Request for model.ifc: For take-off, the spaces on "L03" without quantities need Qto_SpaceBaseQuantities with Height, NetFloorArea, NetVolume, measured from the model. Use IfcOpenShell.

First a look at what the model holds.

```python
import ifcopenshell
import ifcopenshell.util.element
import ifcopenshell.util.unit

model = ifcopenshell.open("model.ifc")
print(model.schema)
for unit_type in ("LENGTHUNIT", "AREAUNIT", "VOLUMEUNIT"):
    print(unit_type, ifcopenshell.util.unit.calculate_unit_scale(model, unit_type))
storey = next(s for s in model.by_type("IfcBuildingStorey") if s.Name == "L03")
spaces = [e for e in ifcopenshell.util.element.get_decomposition(storey) if e.is_a("IfcSpace")]
for e in sorted(spaces, key=lambda e: e.id()):
    print(e.id(), e.is_a(), e.Name, list(ifcopenshell.util.element.get_psets(e, qtos_only=True)), sep=" | ")
```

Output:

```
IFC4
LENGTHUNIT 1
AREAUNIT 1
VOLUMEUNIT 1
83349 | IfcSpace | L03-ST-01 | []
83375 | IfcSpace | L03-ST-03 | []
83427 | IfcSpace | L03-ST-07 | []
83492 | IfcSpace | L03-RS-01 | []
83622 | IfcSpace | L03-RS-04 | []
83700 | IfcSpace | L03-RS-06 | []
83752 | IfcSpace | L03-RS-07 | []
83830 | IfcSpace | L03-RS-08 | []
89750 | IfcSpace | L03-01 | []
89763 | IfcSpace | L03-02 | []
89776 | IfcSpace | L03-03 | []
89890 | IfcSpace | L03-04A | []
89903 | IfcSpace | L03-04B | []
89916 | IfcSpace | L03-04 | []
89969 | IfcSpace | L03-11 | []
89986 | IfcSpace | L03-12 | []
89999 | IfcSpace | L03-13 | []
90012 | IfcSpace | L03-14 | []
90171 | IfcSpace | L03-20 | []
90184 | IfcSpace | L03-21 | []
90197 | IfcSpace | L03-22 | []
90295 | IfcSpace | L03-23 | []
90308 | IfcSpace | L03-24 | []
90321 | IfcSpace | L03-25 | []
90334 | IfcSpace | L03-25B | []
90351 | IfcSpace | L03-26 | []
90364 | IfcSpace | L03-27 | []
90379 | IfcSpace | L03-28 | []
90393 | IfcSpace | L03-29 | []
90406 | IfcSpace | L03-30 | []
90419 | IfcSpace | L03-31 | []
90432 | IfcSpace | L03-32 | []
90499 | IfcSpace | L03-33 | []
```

```python
import ifcopenshell
import ifcopenshell.api.pset
import ifcopenshell.geom
import ifcopenshell.util.element
import ifcopenshell.util.shape
import ifcopenshell.util.unit

model = ifcopenshell.open("model.ifc")
unit_scale = ifcopenshell.util.unit.calculate_unit_scale(model)
area_scale = ifcopenshell.util.unit.calculate_unit_scale(model, "AREAUNIT")
volume_scale = ifcopenshell.util.unit.calculate_unit_scale(model, "VOLUMEUNIT")
settings = ifcopenshell.geom.settings()

storey = next(s for s in model.by_type("IfcBuildingStorey") if s.Name == "L03")
spaces = [e for e in ifcopenshell.util.element.get_decomposition(storey) if e.is_a("IfcSpace")]

for e in sorted(spaces, key=lambda e: e.id()):
    if ifcopenshell.util.element.get_psets(e, qtos_only=True, should_inherit=False):
        continue
    # Geometry comes back in metres, in the element's own axes.
    shape = ifcopenshell.geom.create_shape(settings, e)
    values = {
        "Height": ifcopenshell.util.shape.get_z(shape.geometry) / unit_scale,
        "NetFloorArea": ifcopenshell.util.shape.get_footprint_area(shape.geometry) / area_scale,
        "NetVolume": ifcopenshell.util.shape.get_volume(shape.geometry) / volume_scale,
    }
    qto = ifcopenshell.api.pset.add_qto(model, product=e, name="Qto_SpaceBaseQuantities")
    ifcopenshell.api.pset.edit_qto(model, qto=qto, properties=values)
    print(e.id(), {k: round(v, 3) for k, v in values.items()})

model.write("model_edited.ifc")
```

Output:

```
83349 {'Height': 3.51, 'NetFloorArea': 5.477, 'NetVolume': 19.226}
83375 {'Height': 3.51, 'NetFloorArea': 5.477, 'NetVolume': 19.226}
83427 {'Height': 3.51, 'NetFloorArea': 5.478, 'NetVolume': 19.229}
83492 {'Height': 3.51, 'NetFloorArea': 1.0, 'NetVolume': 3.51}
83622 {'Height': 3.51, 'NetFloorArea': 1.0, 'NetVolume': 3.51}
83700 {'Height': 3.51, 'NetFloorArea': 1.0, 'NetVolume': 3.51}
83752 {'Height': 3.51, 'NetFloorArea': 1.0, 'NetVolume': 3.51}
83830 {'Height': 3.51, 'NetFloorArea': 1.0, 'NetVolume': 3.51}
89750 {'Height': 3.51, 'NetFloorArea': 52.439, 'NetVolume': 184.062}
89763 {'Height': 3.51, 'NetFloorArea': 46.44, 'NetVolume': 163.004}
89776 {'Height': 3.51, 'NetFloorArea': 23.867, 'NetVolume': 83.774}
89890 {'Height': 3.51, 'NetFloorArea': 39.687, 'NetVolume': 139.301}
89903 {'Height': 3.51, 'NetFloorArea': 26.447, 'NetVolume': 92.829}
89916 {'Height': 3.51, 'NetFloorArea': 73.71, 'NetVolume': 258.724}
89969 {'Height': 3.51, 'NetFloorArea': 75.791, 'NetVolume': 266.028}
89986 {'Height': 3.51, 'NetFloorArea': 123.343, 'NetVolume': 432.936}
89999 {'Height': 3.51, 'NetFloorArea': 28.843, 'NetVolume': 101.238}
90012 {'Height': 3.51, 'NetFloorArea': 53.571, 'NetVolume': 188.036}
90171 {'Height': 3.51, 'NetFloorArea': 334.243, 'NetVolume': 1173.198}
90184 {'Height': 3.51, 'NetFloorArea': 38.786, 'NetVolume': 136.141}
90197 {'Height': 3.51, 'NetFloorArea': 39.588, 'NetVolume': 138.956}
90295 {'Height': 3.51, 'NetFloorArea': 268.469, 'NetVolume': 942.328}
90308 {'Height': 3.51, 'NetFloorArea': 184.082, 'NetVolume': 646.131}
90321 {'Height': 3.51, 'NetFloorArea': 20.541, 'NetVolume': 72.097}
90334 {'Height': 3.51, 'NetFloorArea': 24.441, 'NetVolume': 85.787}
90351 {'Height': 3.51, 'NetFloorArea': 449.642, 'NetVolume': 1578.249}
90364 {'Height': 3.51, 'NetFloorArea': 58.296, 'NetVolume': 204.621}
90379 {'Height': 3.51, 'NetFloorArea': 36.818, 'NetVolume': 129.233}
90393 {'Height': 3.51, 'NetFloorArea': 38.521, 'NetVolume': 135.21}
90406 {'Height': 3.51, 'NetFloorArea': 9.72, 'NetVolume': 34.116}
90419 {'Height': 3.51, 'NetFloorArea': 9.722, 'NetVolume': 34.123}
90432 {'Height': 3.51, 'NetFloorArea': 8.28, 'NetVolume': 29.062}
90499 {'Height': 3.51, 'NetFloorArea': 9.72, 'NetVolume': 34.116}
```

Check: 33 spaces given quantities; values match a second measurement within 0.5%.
